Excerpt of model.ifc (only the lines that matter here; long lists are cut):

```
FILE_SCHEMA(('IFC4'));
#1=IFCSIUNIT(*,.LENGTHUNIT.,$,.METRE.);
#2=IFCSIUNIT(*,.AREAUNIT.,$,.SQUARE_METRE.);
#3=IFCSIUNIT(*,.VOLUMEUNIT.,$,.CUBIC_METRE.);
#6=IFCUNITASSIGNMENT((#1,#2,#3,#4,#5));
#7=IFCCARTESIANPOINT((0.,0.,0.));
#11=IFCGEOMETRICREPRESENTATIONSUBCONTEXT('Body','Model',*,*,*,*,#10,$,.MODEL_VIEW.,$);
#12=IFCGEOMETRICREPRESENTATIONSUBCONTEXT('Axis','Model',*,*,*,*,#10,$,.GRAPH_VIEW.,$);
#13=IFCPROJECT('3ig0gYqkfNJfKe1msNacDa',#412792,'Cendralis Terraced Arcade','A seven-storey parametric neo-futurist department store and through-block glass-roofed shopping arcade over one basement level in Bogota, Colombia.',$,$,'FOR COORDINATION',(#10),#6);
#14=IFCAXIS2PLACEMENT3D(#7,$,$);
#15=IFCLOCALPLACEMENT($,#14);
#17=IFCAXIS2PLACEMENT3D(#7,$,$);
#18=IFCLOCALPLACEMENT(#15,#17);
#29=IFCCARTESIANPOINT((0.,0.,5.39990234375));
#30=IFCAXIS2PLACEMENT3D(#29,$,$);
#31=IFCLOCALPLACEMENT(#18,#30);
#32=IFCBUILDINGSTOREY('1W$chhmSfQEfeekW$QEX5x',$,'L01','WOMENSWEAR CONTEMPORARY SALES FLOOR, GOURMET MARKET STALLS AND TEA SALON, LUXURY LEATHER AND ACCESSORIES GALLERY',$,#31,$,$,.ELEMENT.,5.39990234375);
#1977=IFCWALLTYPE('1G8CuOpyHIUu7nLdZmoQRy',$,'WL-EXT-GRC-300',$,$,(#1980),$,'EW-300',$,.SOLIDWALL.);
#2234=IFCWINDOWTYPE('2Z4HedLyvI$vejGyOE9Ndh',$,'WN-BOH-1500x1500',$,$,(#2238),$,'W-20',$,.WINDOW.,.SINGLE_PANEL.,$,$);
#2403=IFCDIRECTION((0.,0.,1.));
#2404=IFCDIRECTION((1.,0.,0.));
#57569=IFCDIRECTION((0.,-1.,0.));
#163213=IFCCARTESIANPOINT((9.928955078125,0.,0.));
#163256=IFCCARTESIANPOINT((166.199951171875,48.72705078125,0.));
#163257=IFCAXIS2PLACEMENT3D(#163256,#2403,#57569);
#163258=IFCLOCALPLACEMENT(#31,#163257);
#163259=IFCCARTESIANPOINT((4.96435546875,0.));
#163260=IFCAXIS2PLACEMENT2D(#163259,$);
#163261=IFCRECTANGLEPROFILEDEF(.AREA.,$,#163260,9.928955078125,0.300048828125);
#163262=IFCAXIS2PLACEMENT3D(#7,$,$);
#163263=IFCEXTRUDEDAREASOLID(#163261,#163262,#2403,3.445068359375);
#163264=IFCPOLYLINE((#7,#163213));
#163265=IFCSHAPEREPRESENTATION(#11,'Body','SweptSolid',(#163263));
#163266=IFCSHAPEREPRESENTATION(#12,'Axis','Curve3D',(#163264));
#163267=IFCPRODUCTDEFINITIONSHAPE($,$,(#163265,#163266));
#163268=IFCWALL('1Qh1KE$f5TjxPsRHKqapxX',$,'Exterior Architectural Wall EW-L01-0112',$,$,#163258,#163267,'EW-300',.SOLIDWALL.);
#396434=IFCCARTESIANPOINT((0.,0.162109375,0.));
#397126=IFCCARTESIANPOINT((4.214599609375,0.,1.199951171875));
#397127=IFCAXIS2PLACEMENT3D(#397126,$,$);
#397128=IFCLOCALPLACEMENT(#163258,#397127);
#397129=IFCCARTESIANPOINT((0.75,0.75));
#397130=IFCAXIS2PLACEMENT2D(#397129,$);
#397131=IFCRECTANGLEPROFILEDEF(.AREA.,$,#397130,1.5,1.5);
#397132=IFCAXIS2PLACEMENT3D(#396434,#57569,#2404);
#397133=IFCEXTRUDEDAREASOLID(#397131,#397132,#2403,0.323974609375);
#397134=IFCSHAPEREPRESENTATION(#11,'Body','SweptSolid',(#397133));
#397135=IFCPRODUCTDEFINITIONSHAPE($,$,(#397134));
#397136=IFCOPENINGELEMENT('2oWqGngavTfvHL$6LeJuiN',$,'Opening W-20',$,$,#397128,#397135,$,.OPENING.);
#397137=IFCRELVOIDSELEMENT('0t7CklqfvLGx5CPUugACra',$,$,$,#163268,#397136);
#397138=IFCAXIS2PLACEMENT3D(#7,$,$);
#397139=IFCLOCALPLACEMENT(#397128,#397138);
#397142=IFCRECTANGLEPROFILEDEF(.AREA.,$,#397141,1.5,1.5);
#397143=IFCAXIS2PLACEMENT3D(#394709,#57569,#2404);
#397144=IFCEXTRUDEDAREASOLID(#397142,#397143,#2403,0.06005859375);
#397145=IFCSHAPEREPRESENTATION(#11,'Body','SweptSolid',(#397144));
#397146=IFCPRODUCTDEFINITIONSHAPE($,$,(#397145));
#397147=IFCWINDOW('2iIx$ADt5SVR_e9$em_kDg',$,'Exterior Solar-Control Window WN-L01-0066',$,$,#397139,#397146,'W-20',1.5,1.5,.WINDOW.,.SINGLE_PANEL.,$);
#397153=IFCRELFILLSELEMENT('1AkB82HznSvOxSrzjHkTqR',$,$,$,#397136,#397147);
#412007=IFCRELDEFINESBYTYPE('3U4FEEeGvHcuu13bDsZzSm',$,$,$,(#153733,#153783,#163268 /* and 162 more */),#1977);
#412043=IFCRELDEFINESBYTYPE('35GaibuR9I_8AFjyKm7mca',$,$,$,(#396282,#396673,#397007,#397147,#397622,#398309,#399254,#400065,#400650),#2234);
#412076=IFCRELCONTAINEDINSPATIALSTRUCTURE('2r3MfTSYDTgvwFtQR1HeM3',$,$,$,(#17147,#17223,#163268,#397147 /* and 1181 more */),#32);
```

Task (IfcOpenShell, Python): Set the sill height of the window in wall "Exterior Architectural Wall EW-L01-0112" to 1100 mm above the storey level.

```python
import numpy as np
import ifcopenshell
import ifcopenshell.api.geometry
import ifcopenshell.geom
import ifcopenshell.util.element
import ifcopenshell.util.placement
import ifcopenshell.util.shape
import ifcopenshell.util.unit

model = ifcopenshell.open("model.ifc")
unit_scale = ifcopenshell.util.unit.calculate_unit_scale(model)

window = model.by_guid("2iIx$ADt5SVR_e9$em_kDg")
opening = window.FillsVoids[0].RelatingOpeningElement
storey = ifcopenshell.util.element.get_container(window, ifc_class="IfcBuildingStorey")
level = ifcopenshell.util.placement.get_local_placement(storey.ObjectPlacement)[2, 3]

# The opening's origin need not be at the sill, so measure its lowest point.
shape = ifcopenshell.geom.create_shape(ifcopenshell.geom.settings(), opening)
bottom = ifcopenshell.util.shape.get_shape_bottom_elevation(shape, shape.geometry) / unit_scale
dz = level + 1.1 / unit_scale - bottom

shift = np.array([0.0, 0.0, dz])
# The window is placed relative to its opening, so it follows when the opening moves.
matrix = ifcopenshell.util.placement.get_local_placement(opening.ObjectPlacement)
matrix[:3, 3] += shift
ifcopenshell.api.geometry.edit_object_placement(
    model, product=opening, matrix=matrix, is_si=False, should_transform_children=True
)

print(f"moved by {dz * unit_scale:+.3f} m")

model.write("model-out.ifc")
```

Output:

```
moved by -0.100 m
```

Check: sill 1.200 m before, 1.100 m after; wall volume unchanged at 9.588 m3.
